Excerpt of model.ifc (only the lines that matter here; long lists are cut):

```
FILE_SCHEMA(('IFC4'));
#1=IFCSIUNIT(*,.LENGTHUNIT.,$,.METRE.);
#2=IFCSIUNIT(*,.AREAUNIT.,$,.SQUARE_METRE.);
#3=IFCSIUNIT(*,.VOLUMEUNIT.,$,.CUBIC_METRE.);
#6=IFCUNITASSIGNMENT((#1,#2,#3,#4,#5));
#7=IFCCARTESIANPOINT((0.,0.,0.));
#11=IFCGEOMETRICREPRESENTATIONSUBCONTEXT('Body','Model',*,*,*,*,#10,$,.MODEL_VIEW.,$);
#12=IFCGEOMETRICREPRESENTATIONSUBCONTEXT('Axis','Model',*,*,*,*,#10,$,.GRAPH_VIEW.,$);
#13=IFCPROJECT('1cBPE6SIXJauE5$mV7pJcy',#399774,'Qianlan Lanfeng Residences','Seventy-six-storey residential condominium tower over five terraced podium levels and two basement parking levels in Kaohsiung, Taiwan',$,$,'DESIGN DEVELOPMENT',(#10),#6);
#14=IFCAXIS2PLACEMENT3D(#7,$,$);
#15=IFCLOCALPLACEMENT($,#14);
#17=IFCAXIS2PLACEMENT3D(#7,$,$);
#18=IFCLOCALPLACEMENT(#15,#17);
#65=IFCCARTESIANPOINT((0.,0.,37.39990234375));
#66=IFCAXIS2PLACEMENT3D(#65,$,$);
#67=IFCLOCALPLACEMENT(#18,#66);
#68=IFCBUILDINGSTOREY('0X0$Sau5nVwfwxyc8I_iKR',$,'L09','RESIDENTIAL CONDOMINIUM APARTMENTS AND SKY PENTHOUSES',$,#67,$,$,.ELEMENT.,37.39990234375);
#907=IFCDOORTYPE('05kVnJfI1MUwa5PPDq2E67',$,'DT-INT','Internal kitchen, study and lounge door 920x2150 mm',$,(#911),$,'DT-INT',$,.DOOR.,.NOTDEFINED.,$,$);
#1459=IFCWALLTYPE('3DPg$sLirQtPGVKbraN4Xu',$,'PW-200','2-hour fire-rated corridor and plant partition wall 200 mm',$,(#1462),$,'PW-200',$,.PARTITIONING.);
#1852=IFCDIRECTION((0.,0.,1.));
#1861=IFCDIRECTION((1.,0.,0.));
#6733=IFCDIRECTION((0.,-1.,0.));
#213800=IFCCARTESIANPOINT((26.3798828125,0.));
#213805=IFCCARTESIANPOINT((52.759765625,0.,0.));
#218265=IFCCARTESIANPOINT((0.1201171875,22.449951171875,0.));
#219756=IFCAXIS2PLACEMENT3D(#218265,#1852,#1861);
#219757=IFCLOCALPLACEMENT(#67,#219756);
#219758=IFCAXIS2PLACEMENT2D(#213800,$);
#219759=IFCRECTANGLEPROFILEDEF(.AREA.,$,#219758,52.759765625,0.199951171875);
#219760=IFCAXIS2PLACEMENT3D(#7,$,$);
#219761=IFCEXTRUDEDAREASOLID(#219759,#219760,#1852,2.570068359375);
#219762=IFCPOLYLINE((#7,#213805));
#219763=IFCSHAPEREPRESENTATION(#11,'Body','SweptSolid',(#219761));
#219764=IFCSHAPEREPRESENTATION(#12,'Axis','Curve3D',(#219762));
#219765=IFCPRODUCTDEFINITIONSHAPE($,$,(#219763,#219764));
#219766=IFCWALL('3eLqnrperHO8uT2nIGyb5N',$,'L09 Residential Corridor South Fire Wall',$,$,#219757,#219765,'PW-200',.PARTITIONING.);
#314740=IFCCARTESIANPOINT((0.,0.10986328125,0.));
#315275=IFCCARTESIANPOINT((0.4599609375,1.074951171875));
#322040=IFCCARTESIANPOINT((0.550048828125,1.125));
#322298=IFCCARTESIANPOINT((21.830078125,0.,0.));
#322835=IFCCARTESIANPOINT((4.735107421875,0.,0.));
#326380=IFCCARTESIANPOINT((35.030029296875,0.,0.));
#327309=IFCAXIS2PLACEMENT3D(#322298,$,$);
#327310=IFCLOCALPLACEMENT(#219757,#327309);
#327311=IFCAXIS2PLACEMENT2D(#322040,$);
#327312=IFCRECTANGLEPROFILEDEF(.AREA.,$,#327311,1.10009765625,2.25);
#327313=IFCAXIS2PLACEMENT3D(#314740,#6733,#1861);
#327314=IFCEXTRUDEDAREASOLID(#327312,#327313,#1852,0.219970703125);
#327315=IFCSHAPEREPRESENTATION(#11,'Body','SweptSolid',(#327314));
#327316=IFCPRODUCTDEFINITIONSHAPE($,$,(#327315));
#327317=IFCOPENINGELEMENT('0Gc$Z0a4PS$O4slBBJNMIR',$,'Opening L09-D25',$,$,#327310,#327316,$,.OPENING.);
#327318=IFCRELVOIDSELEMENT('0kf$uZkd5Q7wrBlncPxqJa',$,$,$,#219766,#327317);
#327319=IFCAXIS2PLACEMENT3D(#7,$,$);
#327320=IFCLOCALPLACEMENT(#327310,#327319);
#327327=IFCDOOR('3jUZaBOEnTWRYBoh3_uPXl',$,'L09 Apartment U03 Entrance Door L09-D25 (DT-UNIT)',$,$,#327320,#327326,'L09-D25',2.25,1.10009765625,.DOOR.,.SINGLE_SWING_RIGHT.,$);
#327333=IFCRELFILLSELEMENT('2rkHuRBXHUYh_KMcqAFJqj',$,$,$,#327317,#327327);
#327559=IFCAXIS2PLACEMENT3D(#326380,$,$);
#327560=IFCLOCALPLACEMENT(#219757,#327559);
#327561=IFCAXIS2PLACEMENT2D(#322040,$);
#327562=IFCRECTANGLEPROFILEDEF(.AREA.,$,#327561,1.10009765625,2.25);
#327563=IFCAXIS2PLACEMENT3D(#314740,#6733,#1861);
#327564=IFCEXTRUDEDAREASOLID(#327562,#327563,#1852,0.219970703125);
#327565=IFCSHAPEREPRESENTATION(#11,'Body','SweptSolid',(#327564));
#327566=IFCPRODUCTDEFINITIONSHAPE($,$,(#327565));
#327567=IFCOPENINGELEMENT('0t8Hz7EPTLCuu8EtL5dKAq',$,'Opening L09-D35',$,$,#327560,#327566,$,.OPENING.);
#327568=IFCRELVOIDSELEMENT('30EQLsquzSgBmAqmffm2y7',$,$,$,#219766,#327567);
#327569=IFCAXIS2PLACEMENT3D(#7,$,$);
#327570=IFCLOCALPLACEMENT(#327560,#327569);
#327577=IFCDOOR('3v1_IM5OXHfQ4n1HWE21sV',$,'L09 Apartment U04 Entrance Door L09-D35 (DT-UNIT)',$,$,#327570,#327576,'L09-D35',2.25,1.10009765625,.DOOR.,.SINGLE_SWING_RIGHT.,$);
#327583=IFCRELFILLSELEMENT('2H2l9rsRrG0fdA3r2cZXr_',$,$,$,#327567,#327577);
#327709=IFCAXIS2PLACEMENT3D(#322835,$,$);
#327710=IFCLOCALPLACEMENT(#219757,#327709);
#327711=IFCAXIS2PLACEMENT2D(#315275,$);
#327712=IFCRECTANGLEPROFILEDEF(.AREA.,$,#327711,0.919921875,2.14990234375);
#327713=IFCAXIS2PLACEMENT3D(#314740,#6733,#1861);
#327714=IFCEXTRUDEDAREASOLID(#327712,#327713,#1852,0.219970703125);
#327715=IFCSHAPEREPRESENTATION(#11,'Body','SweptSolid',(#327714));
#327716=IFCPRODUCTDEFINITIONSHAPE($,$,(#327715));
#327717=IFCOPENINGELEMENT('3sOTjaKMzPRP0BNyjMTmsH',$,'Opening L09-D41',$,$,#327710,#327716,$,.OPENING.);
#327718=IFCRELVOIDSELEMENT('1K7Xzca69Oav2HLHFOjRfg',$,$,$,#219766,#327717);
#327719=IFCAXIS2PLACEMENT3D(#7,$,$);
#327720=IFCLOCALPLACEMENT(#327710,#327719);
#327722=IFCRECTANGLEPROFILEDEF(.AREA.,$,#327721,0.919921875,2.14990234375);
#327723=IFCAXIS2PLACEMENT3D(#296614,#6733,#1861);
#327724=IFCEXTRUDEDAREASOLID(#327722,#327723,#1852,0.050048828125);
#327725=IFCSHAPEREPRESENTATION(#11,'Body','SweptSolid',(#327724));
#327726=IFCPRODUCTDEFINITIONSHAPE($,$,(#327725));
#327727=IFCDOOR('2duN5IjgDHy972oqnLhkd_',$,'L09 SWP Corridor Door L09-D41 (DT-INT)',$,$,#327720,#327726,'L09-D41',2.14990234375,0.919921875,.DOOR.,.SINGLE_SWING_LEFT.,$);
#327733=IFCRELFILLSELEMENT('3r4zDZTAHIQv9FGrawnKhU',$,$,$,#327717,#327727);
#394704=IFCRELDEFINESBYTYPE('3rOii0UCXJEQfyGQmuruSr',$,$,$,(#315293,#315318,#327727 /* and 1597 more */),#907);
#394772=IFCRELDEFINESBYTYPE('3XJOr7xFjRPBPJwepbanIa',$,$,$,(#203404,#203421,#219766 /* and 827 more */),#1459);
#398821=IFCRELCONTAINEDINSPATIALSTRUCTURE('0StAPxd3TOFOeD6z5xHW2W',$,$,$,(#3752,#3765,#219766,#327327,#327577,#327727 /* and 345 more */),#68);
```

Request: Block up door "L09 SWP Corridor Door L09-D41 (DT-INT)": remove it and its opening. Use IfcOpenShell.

```python
import ifcopenshell
import ifcopenshell.api.feature
import ifcopenshell.api.root
import ifcopenshell.geom
import ifcopenshell.util.shape

model = ifcopenshell.open("model.ifc")
settings = ifcopenshell.geom.settings()


def volume(element):
    """Net volume in cubic metres, openings subtracted."""
    shape = ifcopenshell.geom.create_shape(settings, element)
    return ifcopenshell.util.shape.get_volume(shape.geometry)


door = model.by_guid("2duN5IjgDHy972oqnLhkd_")
opening = door.FillsVoids[0].RelatingOpeningElement
wall = opening.VoidsElements[0].RelatingBuildingElement
before = volume(wall)

ifcopenshell.api.root.remove_product(model, product=door)
ifcopenshell.api.feature.remove_feature(model, feature=opening)

after = volume(wall)

print(f"wall volume {before:.3f} -> {after:.3f} m3")

model.write("model_edited.ifc")
```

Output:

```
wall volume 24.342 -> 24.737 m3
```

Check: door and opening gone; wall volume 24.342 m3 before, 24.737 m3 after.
